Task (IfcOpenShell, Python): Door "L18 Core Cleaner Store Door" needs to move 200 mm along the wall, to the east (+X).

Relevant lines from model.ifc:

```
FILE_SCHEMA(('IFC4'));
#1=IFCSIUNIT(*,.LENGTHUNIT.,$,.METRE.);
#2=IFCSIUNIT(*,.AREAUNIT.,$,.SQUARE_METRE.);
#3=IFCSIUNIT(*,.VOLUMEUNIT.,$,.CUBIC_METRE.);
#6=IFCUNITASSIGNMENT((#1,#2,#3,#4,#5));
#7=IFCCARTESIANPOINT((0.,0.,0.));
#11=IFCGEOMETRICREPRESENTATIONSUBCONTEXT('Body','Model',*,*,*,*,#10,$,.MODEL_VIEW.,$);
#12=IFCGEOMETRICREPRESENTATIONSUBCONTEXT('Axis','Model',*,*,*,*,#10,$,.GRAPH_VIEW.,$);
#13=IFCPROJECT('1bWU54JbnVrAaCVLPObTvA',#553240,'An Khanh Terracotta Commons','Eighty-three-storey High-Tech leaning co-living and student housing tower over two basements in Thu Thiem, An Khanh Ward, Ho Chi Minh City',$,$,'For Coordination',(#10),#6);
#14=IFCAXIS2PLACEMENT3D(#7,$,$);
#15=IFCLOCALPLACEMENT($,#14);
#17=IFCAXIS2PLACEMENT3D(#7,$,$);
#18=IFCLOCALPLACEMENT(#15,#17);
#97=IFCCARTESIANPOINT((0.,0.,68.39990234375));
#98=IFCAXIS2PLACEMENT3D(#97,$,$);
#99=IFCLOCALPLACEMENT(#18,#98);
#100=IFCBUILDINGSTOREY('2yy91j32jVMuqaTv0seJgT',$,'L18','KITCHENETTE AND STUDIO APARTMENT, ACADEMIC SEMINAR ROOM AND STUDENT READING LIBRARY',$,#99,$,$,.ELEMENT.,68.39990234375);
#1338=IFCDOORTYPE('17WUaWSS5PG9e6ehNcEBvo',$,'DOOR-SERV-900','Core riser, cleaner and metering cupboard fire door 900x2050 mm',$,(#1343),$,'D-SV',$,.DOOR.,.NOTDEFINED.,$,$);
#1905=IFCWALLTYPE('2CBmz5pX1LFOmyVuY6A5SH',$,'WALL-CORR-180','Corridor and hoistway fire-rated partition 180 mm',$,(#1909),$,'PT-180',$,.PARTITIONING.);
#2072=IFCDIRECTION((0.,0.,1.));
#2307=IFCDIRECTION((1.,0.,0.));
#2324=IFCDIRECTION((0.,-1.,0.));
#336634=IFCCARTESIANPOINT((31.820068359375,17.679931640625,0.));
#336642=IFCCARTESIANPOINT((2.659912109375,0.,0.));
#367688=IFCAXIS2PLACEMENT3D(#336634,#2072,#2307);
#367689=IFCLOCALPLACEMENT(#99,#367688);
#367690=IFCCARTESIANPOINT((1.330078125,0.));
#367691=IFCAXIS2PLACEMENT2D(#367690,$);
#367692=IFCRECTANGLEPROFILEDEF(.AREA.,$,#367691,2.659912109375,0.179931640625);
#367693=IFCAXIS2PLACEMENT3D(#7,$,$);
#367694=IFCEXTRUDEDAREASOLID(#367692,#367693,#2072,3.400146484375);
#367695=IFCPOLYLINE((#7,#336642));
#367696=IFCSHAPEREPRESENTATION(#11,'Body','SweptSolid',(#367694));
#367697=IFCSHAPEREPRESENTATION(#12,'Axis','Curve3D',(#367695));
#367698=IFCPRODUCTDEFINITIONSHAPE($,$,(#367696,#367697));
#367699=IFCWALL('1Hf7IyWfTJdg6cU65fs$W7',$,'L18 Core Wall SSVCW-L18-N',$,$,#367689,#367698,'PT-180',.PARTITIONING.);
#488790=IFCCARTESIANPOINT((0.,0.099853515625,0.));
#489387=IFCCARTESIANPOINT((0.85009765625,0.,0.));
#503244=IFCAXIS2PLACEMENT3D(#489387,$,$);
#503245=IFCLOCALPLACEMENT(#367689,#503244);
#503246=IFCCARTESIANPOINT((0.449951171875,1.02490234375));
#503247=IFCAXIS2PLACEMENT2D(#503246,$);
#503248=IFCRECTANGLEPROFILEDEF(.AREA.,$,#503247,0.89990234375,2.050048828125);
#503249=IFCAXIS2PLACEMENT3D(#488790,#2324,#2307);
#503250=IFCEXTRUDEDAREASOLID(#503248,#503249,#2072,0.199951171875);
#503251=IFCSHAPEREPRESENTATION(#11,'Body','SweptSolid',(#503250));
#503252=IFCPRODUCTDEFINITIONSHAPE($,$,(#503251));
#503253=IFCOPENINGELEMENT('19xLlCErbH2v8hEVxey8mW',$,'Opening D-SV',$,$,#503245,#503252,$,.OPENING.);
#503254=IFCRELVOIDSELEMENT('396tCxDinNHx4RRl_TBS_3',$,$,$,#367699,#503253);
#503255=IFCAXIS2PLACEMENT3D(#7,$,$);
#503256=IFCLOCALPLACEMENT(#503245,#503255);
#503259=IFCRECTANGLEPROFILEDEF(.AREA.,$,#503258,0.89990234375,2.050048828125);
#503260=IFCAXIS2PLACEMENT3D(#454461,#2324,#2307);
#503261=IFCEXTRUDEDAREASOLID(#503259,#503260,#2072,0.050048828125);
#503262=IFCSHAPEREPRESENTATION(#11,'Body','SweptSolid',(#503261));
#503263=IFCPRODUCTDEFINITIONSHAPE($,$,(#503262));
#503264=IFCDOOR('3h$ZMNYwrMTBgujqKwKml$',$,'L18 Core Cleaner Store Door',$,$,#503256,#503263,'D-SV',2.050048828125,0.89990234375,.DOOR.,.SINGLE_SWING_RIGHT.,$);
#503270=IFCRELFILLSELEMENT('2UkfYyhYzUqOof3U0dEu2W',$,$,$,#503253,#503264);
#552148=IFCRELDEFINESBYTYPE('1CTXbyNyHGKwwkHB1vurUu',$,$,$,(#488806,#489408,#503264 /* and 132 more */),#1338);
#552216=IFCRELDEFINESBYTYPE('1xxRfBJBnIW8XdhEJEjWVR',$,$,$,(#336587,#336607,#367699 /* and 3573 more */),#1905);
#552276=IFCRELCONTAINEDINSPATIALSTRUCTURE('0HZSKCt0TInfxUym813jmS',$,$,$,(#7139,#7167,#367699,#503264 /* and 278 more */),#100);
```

```python
import ifcopenshell
import ifcopenshell.api.geometry
import ifcopenshell.util.placement
import ifcopenshell.util.unit

model = ifcopenshell.open("model.ifc")
unit_scale = ifcopenshell.util.unit.calculate_unit_scale(model)

door = model.by_id(503264)
opening = door.FillsVoids[0].RelatingOpeningElement
wall = opening.VoidsElements[0].RelatingBuildingElement

wall_matrix = ifcopenshell.util.placement.get_local_placement(wall.ObjectPlacement)
shift = wall_matrix[:3, 0] * 0.2 / unit_scale
before = ifcopenshell.util.placement.get_local_placement(door.ObjectPlacement)[:3, 3].copy()

# The door is placed relative to its opening, so it follows when the opening moves.
matrix = ifcopenshell.util.placement.get_local_placement(opening.ObjectPlacement)
matrix[:3, 3] += shift
ifcopenshell.api.geometry.edit_object_placement(
    model, product=opening, matrix=matrix, is_si=False, should_transform_children=True
)

after = ifcopenshell.util.placement.get_local_placement(door.ObjectPlacement)[:3, 3]
print("door moved by", (after - before).round(3) + 0.0)

model.write("model_v2.ifc")
```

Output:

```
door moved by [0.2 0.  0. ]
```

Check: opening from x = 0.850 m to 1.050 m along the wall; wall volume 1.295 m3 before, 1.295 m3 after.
